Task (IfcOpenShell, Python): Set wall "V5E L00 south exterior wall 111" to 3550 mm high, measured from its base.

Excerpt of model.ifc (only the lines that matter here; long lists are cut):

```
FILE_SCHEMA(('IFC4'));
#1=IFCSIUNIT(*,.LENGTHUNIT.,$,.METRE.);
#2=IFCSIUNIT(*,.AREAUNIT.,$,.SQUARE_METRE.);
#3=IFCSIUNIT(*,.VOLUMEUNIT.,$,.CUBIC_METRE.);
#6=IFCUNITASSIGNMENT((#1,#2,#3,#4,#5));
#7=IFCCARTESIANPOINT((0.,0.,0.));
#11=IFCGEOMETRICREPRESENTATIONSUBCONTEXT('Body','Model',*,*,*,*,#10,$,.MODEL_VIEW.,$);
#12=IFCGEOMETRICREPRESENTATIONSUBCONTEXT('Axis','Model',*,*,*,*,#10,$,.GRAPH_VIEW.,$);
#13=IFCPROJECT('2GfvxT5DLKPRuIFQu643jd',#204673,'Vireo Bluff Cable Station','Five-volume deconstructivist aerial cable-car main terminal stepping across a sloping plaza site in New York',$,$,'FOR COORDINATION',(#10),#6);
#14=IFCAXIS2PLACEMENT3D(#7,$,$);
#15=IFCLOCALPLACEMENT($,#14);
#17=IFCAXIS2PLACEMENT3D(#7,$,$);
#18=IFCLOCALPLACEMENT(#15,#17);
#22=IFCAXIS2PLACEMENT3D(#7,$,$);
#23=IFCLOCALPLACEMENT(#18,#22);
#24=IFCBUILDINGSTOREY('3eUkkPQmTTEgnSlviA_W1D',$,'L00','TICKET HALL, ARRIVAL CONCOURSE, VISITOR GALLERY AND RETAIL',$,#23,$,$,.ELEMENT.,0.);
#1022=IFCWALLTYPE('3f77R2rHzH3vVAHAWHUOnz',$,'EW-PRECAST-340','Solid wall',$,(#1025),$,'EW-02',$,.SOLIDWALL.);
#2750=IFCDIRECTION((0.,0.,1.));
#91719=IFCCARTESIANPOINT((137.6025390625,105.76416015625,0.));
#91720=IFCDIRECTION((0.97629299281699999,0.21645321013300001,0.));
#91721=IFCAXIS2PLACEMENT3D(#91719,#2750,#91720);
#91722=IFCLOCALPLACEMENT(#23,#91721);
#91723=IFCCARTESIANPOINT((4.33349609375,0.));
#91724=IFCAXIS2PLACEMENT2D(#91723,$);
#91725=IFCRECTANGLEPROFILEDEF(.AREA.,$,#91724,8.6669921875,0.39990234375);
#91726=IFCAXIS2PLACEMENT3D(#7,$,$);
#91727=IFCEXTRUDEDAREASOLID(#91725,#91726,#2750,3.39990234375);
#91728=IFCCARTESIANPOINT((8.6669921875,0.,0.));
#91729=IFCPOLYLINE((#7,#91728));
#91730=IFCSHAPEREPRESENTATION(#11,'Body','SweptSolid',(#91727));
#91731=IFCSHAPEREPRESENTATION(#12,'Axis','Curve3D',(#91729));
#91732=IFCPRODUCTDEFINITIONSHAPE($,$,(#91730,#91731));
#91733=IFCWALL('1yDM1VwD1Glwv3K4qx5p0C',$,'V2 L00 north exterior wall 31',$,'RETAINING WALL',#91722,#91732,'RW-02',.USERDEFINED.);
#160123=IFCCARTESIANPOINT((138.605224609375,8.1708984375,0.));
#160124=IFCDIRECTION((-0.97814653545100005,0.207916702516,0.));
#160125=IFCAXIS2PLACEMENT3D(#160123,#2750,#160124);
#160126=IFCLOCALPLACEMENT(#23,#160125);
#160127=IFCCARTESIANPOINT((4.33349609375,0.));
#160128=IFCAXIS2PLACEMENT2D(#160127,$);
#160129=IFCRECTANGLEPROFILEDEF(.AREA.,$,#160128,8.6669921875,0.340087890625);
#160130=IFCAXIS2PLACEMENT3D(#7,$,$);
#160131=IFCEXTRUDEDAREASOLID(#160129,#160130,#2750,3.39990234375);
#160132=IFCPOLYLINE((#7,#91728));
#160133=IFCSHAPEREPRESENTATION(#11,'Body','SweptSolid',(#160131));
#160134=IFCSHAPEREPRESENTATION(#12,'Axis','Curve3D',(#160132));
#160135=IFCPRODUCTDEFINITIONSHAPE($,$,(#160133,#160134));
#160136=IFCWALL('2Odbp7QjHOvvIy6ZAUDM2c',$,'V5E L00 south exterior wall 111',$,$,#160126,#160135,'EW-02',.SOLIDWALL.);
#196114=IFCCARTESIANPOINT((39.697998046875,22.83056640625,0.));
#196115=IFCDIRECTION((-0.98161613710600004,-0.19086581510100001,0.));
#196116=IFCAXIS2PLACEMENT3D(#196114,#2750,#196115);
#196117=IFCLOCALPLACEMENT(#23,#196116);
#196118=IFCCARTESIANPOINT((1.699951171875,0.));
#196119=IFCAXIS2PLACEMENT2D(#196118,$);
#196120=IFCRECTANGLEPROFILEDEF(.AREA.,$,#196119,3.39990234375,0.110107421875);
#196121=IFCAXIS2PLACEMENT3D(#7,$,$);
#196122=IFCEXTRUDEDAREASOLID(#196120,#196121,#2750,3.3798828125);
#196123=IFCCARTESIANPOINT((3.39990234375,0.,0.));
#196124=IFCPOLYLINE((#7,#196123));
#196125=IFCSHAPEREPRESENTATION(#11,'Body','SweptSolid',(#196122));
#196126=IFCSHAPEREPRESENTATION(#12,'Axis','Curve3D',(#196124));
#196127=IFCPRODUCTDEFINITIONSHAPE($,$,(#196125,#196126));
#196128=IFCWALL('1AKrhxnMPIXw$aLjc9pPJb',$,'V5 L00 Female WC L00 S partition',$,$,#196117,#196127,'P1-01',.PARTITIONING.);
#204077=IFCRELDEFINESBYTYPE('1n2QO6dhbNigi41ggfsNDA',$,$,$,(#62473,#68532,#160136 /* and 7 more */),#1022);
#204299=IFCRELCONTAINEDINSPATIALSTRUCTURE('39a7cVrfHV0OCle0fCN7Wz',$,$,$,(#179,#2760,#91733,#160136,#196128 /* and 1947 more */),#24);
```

```python
import ifcopenshell
import ifcopenshell.geom
import ifcopenshell.util.representation
import ifcopenshell.util.shape
import ifcopenshell.util.unit

model = ifcopenshell.open("model.ifc")
unit_scale = ifcopenshell.util.unit.calculate_unit_scale(model)
settings = ifcopenshell.geom.settings()


def volume(element):
    """Net volume in cubic metres, openings subtracted."""
    shape = ifcopenshell.geom.create_shape(settings, element)
    return ifcopenshell.util.shape.get_volume(shape.geometry)


wall = model.by_id(160136)
before = volume(wall)

body = ifcopenshell.util.representation.get_representation(wall, "Model", "Body")
solid = body.Items[0]
old_height = solid.Depth
solid.Depth = 3.55 / unit_scale
after = volume(wall)

print(f"height {old_height:g} -> {solid.Depth:g}, volume {before:.3f} -> {after:.3f} m3")

model.write("model_v2.ifc")
```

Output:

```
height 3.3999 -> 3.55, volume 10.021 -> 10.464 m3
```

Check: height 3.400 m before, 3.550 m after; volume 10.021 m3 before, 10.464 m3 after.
